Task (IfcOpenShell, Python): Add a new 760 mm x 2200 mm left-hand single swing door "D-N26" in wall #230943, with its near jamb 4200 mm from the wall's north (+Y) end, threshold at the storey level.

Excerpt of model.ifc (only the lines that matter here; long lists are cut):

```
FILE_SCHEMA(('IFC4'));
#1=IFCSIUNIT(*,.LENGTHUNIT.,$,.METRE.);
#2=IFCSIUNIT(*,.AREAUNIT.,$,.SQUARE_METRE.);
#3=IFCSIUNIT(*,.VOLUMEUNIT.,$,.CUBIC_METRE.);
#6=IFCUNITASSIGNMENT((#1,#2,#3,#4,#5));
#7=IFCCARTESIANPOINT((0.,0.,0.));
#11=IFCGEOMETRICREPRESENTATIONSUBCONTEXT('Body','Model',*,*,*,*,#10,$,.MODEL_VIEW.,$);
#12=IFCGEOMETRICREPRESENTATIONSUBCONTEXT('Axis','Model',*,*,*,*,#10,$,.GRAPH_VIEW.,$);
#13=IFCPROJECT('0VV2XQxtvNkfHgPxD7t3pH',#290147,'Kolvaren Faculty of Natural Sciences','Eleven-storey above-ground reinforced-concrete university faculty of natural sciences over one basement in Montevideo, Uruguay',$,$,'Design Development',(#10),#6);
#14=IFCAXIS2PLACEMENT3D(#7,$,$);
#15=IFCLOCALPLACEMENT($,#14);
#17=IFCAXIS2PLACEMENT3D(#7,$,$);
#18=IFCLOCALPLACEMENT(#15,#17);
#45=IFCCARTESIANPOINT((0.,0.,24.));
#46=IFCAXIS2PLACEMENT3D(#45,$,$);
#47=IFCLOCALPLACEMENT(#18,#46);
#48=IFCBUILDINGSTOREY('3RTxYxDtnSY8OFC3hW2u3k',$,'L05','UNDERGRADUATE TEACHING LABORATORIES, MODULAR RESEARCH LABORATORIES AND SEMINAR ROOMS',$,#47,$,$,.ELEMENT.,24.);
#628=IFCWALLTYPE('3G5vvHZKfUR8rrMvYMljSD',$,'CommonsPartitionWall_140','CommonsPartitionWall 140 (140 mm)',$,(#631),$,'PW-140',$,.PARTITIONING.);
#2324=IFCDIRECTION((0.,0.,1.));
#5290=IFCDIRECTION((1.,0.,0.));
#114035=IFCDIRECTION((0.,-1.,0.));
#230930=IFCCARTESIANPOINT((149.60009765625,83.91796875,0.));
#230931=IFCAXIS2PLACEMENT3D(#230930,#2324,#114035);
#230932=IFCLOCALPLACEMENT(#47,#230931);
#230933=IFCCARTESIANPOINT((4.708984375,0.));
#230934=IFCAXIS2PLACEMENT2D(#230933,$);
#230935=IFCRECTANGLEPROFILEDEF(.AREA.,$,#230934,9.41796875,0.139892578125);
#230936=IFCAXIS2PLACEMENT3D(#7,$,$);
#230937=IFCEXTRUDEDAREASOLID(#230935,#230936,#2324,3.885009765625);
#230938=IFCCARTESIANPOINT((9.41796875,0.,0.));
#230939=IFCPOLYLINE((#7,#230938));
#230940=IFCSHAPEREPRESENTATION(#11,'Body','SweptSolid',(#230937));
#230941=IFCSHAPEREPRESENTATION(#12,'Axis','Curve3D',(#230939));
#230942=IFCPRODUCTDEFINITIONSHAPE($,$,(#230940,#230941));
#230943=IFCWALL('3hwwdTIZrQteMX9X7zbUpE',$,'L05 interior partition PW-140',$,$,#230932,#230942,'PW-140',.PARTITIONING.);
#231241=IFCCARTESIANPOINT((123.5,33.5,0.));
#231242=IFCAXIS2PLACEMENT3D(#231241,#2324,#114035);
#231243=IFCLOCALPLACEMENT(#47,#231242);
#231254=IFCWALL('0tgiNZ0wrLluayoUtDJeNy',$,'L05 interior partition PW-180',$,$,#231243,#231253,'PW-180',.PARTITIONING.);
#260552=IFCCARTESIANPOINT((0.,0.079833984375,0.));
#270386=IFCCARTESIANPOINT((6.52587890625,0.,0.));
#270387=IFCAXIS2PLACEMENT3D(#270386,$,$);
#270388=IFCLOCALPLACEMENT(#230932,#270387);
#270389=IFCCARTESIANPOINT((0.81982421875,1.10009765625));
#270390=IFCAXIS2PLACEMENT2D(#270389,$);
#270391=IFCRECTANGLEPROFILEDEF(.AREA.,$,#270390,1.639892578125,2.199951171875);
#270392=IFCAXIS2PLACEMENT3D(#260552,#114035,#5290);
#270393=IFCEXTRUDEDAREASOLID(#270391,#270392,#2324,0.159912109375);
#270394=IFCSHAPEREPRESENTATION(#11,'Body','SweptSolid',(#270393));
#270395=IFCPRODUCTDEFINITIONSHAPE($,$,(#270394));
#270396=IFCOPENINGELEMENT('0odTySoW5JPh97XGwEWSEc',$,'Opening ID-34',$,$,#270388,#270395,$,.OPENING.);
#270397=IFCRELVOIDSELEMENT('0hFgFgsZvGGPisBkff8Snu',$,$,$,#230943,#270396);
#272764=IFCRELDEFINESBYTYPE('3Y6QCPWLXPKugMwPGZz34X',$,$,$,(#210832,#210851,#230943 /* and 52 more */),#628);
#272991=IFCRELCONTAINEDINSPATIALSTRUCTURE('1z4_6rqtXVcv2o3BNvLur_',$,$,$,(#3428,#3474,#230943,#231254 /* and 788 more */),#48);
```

```python
import numpy as np
import ifcopenshell
import ifcopenshell.api.feature
import ifcopenshell.api.geometry
import ifcopenshell.api.root
import ifcopenshell.api.spatial
import ifcopenshell.geom
import ifcopenshell.util.element
import ifcopenshell.util.placement
import ifcopenshell.util.representation
import ifcopenshell.util.shape
import ifcopenshell.util.unit

model = ifcopenshell.open("model.ifc")
unit_scale = ifcopenshell.util.unit.calculate_unit_scale(model)
settings = ifcopenshell.geom.settings()


def volume(element):
    """Net volume in cubic metres, openings subtracted."""
    shape = ifcopenshell.geom.create_shape(settings, element)
    return ifcopenshell.util.shape.get_volume(shape.geometry)


wall = model.by_guid("3hwwdTIZrQteMX9X7zbUpE")
storey = ifcopenshell.util.element.get_container(wall, ifc_class="IfcBuildingStorey")
context = ifcopenshell.util.representation.get_context(model, "Model", "Body", "MODEL_VIEW")
before = volume(wall)

width, height, from_end, sill = 0.76, 2.2, 4.2, 0.0  # metres

# The wall runs along its own X axis, and the end named is its -X end.
wall_shape = ifcopenshell.geom.create_shape(settings, wall)
x, y, z = ifcopenshell.util.shape.get_vertices(wall_shape.geometry).T
start = x.min() + from_end
face, thickness = float(y.min()), float(y.max() - y.min())
wall_matrix = ifcopenshell.util.placement.get_local_placement(wall.ObjectPlacement)
level = ifcopenshell.util.placement.get_local_placement(storey.ObjectPlacement)[2, 3]


def in_wall(x, y):
    """Placement at x, y metres in the wall's axes, at sill height."""
    matrix = wall_matrix.copy()
    matrix[:, 3] = wall_matrix @ np.array([x / unit_scale, y / unit_scale, 0.0, 1.0])
    matrix[2, 3] = level + sill / unit_scale
    return matrix


# Opening: a box that overshoots both wall faces by 50 mm.
opening = ifcopenshell.api.root.create_entity(model, ifc_class="IfcOpeningElement", predefined_type="OPENING")
box = ifcopenshell.api.geometry.add_wall_representation(
    model, context=context, length=width, height=height, thickness=thickness + 0.1
)
ifcopenshell.api.geometry.assign_representation(model, product=opening, representation=box)
ifcopenshell.api.geometry.edit_object_placement(model, product=opening, matrix=in_wall(start, face - 0.05), is_si=False)
ifcopenshell.api.feature.add_feature(model, feature=opening, element=wall)

door = ifcopenshell.api.root.create_entity(model, ifc_class="IfcDoor", name="D-N26", predefined_type="DOOR")
door.OverallWidth, door.OverallHeight = width / unit_scale, height / unit_scale
door.OperationType = "SINGLE_SWING_LEFT"
body = ifcopenshell.api.geometry.add_door_representation(
    model,
    context=context,
    overall_width=door.OverallWidth,
    overall_height=door.OverallHeight,
    operation_type="SINGLE_SWING_LEFT",
    lining_properties={"LiningDepth": thickness / unit_scale, "ThresholdDepth": thickness / unit_scale},
)
ifcopenshell.api.geometry.assign_representation(model, product=door, representation=body)
ifcopenshell.api.spatial.assign_container(model, products=[door], relating_structure=storey)
ifcopenshell.api.feature.add_filling(model, opening=opening, element=door)

# The lining spans the wall, so the door starts at the wall face.
ifcopenshell.api.geometry.edit_object_placement(model, product=door, matrix=in_wall(start, face), is_si=False)

after = volume(wall)

print(f"wall volume {before:.3f} -> {after:.3f} m3")

model.write("model_edited.ifc")
```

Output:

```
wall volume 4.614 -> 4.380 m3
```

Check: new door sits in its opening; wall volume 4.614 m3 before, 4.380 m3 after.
